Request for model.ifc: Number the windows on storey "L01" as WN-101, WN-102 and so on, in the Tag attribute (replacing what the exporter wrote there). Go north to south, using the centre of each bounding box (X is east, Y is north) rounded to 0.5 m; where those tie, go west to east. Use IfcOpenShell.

First a look at what the model holds.

```python
import ifcopenshell
import ifcopenshell.util.element
import ifcopenshell.util.placement

model = ifcopenshell.open("model.ifc")
print(model.schema)
storey = next(s for s in model.by_type("IfcBuildingStorey") if s.Name == "L01")
windows = [e for e in ifcopenshell.util.element.get_decomposition(storey) if e.is_a("IfcWindow")]
for e in sorted(windows, key=lambda e: e.id()):
    origin = ifcopenshell.util.placement.get_local_placement(e.ObjectPlacement)[:3, 3]
    print(e.id(), e.Tag, e.Name, origin.round(2) + 0.0, sep=" | ")
```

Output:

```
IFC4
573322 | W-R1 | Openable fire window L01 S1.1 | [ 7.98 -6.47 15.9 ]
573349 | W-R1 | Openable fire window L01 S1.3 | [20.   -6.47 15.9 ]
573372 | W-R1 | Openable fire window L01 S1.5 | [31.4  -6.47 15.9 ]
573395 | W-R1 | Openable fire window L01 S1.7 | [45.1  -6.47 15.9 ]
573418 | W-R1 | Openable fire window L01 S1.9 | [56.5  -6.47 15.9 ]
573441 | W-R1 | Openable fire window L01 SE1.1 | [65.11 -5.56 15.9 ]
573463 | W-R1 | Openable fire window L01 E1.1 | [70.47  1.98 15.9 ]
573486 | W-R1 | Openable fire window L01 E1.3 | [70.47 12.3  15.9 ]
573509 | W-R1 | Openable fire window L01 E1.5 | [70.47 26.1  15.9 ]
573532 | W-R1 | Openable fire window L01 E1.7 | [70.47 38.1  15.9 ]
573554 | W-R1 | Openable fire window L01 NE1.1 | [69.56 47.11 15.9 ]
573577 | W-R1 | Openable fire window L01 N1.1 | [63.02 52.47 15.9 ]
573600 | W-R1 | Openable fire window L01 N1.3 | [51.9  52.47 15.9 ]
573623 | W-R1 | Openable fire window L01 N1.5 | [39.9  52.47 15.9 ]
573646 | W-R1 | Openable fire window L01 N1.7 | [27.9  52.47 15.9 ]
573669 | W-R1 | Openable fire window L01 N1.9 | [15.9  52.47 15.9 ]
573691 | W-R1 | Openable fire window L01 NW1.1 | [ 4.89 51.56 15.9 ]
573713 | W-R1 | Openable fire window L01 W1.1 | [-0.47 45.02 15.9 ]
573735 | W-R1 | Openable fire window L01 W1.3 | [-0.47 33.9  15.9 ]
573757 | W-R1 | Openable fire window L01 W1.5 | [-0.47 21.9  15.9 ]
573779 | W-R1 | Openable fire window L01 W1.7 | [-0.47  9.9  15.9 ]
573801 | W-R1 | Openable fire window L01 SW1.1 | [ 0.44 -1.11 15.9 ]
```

```python
import ifcopenshell
import ifcopenshell.geom
import ifcopenshell.util.element
import ifcopenshell.util.shape

model = ifcopenshell.open("model.ifc")
settings = ifcopenshell.geom.settings()
settings.set("use-world-coords", True)


def centre(element):
    shape = ifcopenshell.geom.create_shape(settings, element)
    return ifcopenshell.util.shape.get_bbox_centroid(shape.geometry)


storey = next(s for s in model.by_type("IfcBuildingStorey") if s.Name == "L01")
windows = [e for e in ifcopenshell.util.element.get_decomposition(storey) if e.is_a("IfcWindow")]

# Insertion points can sit at a corner or the storey origin, so sort by the geometry (in metres).
centres = {e: centre(e) for e in windows}
windows.sort(key=lambda e: (-round(centres[e][1] / 0.5), centres[e][0]))

for i, e in enumerate(windows, start=1):
    number = f"WN-1{i:02d}"
    e.Tag = number
    print(e.id(), number)

model.write("model_edited.ifc")
```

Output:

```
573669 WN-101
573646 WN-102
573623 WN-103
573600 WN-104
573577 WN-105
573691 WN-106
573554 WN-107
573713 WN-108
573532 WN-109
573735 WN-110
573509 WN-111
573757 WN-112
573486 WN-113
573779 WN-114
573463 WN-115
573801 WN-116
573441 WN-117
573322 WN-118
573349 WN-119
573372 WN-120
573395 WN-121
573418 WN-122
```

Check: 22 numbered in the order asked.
